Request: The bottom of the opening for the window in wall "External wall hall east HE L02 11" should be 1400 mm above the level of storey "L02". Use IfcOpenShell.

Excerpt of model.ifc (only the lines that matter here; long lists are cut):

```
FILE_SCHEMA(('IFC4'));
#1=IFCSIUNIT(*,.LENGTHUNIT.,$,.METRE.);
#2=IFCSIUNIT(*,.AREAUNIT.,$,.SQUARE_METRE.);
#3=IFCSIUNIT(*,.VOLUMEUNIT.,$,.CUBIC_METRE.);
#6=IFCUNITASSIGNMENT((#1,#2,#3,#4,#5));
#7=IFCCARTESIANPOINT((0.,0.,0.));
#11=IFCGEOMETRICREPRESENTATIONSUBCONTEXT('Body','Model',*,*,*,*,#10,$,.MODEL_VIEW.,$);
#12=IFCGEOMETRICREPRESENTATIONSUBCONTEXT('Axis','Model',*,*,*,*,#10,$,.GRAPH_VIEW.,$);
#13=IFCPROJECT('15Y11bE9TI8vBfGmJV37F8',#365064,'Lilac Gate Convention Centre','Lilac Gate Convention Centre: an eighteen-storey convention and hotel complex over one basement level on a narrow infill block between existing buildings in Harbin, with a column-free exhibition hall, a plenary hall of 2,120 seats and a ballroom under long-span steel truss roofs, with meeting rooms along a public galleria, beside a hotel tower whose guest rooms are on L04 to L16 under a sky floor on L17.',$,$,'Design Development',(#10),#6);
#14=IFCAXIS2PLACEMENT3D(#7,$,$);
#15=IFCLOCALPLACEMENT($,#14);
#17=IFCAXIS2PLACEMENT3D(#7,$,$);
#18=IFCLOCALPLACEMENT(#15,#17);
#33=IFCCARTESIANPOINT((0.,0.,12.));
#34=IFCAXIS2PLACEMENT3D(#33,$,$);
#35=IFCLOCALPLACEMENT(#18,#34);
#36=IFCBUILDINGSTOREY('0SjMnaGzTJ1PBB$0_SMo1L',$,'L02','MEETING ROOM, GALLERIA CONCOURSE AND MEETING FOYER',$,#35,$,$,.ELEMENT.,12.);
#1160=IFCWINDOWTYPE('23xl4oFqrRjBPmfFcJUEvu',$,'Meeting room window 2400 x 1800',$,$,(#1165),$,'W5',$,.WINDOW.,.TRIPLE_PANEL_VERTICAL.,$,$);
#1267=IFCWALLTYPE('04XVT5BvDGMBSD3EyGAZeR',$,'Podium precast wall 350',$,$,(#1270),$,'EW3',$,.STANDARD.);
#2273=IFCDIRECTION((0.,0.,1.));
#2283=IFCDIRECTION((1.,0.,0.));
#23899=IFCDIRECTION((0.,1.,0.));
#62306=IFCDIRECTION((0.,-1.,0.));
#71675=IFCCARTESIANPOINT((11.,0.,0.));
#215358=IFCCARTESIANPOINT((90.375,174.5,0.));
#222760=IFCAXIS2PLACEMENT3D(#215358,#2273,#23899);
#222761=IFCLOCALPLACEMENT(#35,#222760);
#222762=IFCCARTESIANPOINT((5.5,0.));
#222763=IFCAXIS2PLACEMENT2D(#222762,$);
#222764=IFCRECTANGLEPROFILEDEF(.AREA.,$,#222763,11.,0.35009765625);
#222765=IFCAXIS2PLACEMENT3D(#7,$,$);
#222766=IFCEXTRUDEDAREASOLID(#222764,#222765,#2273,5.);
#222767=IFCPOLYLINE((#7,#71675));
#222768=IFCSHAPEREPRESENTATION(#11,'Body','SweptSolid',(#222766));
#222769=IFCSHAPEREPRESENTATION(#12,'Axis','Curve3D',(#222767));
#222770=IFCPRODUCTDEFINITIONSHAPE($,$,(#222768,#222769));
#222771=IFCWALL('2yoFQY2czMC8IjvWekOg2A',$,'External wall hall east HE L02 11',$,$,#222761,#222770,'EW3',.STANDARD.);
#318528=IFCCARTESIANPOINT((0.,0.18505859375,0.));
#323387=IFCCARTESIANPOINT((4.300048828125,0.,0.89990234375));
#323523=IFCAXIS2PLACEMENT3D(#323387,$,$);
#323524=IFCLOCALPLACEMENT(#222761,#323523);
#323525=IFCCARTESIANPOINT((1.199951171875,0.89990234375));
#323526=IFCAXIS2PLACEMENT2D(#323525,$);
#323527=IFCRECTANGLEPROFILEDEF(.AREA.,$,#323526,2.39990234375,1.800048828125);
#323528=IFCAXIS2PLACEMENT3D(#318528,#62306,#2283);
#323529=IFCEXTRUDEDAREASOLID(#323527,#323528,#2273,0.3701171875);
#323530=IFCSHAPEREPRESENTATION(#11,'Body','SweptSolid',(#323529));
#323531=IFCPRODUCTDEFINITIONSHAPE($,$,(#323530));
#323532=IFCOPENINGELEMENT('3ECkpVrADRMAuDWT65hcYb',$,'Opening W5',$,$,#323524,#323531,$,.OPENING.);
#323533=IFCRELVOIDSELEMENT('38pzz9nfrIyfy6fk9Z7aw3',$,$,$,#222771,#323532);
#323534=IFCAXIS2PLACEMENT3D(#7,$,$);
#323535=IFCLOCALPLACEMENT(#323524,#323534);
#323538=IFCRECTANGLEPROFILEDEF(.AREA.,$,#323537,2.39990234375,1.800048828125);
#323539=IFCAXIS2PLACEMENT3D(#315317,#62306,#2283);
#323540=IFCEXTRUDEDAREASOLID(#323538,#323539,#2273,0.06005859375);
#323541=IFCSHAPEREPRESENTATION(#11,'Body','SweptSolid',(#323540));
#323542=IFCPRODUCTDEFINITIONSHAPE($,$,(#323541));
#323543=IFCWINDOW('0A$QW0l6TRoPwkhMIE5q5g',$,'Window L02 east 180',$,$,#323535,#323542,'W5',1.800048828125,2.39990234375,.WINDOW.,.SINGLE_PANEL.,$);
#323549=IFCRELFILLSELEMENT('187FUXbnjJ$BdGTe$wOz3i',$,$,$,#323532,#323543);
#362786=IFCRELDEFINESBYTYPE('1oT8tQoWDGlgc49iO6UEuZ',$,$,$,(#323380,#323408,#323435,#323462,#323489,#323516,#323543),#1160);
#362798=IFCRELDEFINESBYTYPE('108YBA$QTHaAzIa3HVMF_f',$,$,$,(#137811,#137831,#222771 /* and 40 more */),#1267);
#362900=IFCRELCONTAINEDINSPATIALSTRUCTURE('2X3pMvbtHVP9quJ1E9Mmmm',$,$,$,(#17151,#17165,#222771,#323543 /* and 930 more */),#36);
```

```python
import numpy as np
import ifcopenshell
import ifcopenshell.api.geometry
import ifcopenshell.geom
import ifcopenshell.util.element
import ifcopenshell.util.placement
import ifcopenshell.util.shape
import ifcopenshell.util.unit

model = ifcopenshell.open("model.ifc")
unit_scale = ifcopenshell.util.unit.calculate_unit_scale(model)

window = model.by_guid("0A$QW0l6TRoPwkhMIE5q5g")
opening = window.FillsVoids[0].RelatingOpeningElement
storey = ifcopenshell.util.element.get_container(window, ifc_class="IfcBuildingStorey")
level = ifcopenshell.util.placement.get_local_placement(storey.ObjectPlacement)[2, 3]

# The opening's origin need not be at the sill, so measure its lowest point.
shape = ifcopenshell.geom.create_shape(ifcopenshell.geom.settings(), opening)
bottom = ifcopenshell.util.shape.get_shape_bottom_elevation(shape, shape.geometry) / unit_scale
dz = level + 1.4 / unit_scale - bottom

shift = np.array([0.0, 0.0, dz])
# The window is placed relative to its opening, so it follows when the opening moves.
matrix = ifcopenshell.util.placement.get_local_placement(opening.ObjectPlacement)
matrix[:3, 3] += shift
ifcopenshell.api.geometry.edit_object_placement(
    model, product=opening, matrix=matrix, is_si=False, should_transform_children=True
)

print(f"moved by {dz * unit_scale:+.3f} m")

model.write("model_rev.ifc")
```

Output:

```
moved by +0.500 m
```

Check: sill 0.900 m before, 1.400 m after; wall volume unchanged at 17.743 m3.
